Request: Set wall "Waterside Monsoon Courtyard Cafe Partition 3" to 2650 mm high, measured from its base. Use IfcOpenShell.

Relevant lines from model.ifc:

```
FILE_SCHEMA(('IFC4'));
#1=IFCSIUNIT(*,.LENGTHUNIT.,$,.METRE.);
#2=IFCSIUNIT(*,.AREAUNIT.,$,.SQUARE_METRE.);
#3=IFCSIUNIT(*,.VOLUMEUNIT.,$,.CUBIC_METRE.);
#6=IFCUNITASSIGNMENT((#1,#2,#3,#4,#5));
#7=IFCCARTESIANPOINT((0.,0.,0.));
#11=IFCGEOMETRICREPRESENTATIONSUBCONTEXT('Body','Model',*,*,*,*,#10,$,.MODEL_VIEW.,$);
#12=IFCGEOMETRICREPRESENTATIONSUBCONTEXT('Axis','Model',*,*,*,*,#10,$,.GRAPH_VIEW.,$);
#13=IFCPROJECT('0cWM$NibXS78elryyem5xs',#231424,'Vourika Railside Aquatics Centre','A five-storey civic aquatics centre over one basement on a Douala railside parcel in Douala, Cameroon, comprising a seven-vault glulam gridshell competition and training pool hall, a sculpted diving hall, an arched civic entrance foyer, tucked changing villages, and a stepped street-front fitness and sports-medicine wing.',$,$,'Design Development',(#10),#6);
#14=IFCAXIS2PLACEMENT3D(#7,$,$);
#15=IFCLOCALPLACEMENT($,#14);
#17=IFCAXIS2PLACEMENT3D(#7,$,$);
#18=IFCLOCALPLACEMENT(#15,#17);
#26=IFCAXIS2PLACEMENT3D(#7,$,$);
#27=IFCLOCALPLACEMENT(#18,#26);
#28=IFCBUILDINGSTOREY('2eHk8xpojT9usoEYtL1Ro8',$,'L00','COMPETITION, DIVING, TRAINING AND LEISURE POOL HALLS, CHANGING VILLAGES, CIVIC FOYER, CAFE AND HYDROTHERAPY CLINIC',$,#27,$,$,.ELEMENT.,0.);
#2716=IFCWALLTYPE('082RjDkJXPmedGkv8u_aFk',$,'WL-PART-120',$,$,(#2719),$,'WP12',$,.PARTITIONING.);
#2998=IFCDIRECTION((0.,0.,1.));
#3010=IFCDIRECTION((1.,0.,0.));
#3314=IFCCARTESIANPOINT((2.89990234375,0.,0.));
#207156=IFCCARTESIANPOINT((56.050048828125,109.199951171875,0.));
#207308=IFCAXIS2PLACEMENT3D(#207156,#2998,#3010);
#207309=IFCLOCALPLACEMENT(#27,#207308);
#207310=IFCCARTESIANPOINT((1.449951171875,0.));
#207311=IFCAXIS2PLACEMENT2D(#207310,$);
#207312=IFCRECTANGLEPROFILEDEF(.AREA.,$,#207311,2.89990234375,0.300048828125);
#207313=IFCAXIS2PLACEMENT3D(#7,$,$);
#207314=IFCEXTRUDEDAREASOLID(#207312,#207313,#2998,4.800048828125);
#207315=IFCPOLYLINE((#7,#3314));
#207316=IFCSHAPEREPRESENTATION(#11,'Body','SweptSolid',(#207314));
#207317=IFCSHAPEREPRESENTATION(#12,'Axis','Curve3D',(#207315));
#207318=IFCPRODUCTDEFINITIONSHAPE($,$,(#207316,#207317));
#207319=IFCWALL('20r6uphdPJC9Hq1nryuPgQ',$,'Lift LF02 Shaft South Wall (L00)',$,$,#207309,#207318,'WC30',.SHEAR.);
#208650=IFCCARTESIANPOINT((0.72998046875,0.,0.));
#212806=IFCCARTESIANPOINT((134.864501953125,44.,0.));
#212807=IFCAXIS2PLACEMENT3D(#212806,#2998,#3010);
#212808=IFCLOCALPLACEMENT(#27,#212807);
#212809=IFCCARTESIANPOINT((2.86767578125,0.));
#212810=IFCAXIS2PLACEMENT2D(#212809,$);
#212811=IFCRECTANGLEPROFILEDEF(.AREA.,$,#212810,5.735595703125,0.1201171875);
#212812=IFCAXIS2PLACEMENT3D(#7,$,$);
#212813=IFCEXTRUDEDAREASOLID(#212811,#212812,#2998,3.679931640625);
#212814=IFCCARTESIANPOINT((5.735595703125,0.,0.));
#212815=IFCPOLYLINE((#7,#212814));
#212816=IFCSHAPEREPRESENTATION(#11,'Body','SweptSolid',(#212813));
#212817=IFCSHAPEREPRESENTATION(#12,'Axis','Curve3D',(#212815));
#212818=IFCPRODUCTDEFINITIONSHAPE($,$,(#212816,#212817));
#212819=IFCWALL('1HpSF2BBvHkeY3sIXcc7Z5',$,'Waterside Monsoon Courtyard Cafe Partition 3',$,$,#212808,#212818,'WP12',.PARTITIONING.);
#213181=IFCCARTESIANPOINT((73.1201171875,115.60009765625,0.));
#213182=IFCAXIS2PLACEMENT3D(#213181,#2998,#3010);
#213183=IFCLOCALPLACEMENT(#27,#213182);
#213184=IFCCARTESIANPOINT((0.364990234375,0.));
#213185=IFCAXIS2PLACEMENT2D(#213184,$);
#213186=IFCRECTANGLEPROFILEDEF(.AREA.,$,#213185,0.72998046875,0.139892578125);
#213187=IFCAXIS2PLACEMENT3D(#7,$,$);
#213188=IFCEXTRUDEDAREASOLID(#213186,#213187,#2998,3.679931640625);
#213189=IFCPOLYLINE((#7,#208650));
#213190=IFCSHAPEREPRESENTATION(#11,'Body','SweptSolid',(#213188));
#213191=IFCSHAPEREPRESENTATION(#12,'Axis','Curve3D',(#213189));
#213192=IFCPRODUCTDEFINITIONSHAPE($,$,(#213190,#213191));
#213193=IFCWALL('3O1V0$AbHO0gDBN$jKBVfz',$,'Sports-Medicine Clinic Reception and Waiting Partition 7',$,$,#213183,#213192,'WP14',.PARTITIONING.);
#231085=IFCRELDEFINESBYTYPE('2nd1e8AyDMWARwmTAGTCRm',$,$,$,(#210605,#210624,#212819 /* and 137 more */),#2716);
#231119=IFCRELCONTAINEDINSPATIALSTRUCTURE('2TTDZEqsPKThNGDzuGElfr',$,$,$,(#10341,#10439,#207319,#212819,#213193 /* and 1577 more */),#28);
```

```python
import ifcopenshell
import ifcopenshell.geom
import ifcopenshell.util.representation
import ifcopenshell.util.shape
import ifcopenshell.util.unit

model = ifcopenshell.open("model.ifc")
unit_scale = ifcopenshell.util.unit.calculate_unit_scale(model)
settings = ifcopenshell.geom.settings()


def volume(element):
    """Net volume in cubic metres, openings subtracted."""
    shape = ifcopenshell.geom.create_shape(settings, element)
    return ifcopenshell.util.shape.get_volume(shape.geometry)


wall = model.by_guid("1HpSF2BBvHkeY3sIXcc7Z5")
before = volume(wall)

body = ifcopenshell.util.representation.get_representation(wall, "Model", "Body")
solid = body.Items[0]
old_height = solid.Depth
solid.Depth = 2.65 / unit_scale
after = volume(wall)

print(f"height {old_height:g} -> {solid.Depth:g}, volume {before:.3f} -> {after:.3f} m3")

model.write("model_v2.ifc")
```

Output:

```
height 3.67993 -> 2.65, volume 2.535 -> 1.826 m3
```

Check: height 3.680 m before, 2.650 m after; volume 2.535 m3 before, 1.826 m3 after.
